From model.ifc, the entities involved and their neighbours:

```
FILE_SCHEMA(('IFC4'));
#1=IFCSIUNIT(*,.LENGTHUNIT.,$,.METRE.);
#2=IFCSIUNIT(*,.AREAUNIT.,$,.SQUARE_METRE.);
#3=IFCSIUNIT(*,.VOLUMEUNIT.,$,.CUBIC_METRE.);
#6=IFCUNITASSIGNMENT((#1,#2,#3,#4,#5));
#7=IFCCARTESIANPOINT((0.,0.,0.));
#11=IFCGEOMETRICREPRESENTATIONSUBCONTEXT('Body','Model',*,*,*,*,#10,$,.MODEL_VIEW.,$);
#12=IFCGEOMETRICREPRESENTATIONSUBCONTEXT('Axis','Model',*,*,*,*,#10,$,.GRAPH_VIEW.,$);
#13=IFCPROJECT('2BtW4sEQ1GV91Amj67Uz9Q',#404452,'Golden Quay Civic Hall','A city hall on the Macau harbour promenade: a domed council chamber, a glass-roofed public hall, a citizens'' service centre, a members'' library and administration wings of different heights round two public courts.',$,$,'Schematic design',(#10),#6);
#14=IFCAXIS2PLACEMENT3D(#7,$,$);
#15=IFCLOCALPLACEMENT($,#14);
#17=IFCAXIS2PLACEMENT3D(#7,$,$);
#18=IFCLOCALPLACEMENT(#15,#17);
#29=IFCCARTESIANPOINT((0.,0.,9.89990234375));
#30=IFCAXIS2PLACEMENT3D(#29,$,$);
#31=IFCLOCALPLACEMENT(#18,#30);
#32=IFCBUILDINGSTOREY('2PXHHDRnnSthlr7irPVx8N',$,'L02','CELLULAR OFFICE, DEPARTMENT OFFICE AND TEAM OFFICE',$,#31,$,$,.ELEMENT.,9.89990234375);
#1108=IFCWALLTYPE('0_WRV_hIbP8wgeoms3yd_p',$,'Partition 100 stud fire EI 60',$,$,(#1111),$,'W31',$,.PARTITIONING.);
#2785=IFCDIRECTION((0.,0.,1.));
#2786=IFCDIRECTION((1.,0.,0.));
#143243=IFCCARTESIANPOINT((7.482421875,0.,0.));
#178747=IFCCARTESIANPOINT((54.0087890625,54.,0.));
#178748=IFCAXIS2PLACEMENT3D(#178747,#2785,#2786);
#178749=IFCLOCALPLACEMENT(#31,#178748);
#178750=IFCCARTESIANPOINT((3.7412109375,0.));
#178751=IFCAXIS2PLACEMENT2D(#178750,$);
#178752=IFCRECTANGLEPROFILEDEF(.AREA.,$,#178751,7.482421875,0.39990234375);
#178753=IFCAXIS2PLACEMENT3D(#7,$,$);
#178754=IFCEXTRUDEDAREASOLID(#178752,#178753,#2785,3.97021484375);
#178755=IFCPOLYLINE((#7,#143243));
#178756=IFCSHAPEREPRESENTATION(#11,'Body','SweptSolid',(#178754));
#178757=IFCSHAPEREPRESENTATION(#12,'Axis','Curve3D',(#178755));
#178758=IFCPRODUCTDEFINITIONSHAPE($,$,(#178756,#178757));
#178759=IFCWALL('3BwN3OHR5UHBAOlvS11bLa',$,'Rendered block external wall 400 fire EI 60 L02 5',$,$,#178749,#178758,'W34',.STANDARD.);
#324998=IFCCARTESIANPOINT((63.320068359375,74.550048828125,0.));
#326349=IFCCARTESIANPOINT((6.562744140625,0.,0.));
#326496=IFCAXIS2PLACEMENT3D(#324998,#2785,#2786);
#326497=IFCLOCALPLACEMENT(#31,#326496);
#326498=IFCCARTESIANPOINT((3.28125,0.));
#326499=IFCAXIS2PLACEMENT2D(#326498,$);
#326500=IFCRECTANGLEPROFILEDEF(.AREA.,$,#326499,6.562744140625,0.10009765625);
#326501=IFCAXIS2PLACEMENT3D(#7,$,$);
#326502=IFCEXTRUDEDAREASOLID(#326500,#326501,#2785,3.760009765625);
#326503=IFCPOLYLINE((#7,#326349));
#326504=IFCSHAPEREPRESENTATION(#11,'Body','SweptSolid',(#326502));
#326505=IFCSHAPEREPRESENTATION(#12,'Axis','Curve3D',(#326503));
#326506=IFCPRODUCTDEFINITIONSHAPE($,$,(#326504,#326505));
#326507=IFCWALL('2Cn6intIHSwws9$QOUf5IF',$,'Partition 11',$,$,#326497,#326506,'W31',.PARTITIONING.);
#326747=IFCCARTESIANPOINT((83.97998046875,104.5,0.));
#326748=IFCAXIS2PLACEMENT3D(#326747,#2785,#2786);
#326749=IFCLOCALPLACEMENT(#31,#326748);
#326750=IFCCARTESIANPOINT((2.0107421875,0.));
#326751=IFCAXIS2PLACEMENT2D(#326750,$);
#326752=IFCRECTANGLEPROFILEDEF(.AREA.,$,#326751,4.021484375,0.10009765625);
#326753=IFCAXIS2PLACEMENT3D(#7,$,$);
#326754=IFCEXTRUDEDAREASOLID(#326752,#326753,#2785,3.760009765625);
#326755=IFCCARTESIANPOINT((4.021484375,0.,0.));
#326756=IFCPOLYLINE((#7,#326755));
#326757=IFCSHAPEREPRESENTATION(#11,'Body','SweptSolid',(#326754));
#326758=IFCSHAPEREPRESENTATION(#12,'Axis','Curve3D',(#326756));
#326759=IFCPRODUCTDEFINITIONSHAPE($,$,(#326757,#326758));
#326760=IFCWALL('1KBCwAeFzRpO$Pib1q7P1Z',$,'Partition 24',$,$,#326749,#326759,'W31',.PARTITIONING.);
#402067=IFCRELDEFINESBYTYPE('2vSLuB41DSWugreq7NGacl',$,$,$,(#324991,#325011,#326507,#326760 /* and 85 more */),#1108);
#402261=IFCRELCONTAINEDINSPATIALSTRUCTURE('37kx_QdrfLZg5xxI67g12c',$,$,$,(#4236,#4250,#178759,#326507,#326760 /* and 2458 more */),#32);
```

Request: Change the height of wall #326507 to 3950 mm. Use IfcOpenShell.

```python
import ifcopenshell
import ifcopenshell.geom
import ifcopenshell.util.representation
import ifcopenshell.util.shape
import ifcopenshell.util.unit

model = ifcopenshell.open("model.ifc")
unit_scale = ifcopenshell.util.unit.calculate_unit_scale(model)
settings = ifcopenshell.geom.settings()


def volume(element):
    """Net volume in cubic metres, openings subtracted."""
    shape = ifcopenshell.geom.create_shape(settings, element)
    return ifcopenshell.util.shape.get_volume(shape.geometry)


wall = model.by_guid("2Cn6intIHSwws9$QOUf5IF")
before = volume(wall)

body = ifcopenshell.util.representation.get_representation(wall, "Model", "Body")
solid = body.Items[0]
old_height = solid.Depth
solid.Depth = 3.95 / unit_scale
after = volume(wall)

print(f"height {old_height:g} -> {solid.Depth:g}, volume {before:.3f} -> {after:.3f} m3")

model.write("model_v2.ifc")
```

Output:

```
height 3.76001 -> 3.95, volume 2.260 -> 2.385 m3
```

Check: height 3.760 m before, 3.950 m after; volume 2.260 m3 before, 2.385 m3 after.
